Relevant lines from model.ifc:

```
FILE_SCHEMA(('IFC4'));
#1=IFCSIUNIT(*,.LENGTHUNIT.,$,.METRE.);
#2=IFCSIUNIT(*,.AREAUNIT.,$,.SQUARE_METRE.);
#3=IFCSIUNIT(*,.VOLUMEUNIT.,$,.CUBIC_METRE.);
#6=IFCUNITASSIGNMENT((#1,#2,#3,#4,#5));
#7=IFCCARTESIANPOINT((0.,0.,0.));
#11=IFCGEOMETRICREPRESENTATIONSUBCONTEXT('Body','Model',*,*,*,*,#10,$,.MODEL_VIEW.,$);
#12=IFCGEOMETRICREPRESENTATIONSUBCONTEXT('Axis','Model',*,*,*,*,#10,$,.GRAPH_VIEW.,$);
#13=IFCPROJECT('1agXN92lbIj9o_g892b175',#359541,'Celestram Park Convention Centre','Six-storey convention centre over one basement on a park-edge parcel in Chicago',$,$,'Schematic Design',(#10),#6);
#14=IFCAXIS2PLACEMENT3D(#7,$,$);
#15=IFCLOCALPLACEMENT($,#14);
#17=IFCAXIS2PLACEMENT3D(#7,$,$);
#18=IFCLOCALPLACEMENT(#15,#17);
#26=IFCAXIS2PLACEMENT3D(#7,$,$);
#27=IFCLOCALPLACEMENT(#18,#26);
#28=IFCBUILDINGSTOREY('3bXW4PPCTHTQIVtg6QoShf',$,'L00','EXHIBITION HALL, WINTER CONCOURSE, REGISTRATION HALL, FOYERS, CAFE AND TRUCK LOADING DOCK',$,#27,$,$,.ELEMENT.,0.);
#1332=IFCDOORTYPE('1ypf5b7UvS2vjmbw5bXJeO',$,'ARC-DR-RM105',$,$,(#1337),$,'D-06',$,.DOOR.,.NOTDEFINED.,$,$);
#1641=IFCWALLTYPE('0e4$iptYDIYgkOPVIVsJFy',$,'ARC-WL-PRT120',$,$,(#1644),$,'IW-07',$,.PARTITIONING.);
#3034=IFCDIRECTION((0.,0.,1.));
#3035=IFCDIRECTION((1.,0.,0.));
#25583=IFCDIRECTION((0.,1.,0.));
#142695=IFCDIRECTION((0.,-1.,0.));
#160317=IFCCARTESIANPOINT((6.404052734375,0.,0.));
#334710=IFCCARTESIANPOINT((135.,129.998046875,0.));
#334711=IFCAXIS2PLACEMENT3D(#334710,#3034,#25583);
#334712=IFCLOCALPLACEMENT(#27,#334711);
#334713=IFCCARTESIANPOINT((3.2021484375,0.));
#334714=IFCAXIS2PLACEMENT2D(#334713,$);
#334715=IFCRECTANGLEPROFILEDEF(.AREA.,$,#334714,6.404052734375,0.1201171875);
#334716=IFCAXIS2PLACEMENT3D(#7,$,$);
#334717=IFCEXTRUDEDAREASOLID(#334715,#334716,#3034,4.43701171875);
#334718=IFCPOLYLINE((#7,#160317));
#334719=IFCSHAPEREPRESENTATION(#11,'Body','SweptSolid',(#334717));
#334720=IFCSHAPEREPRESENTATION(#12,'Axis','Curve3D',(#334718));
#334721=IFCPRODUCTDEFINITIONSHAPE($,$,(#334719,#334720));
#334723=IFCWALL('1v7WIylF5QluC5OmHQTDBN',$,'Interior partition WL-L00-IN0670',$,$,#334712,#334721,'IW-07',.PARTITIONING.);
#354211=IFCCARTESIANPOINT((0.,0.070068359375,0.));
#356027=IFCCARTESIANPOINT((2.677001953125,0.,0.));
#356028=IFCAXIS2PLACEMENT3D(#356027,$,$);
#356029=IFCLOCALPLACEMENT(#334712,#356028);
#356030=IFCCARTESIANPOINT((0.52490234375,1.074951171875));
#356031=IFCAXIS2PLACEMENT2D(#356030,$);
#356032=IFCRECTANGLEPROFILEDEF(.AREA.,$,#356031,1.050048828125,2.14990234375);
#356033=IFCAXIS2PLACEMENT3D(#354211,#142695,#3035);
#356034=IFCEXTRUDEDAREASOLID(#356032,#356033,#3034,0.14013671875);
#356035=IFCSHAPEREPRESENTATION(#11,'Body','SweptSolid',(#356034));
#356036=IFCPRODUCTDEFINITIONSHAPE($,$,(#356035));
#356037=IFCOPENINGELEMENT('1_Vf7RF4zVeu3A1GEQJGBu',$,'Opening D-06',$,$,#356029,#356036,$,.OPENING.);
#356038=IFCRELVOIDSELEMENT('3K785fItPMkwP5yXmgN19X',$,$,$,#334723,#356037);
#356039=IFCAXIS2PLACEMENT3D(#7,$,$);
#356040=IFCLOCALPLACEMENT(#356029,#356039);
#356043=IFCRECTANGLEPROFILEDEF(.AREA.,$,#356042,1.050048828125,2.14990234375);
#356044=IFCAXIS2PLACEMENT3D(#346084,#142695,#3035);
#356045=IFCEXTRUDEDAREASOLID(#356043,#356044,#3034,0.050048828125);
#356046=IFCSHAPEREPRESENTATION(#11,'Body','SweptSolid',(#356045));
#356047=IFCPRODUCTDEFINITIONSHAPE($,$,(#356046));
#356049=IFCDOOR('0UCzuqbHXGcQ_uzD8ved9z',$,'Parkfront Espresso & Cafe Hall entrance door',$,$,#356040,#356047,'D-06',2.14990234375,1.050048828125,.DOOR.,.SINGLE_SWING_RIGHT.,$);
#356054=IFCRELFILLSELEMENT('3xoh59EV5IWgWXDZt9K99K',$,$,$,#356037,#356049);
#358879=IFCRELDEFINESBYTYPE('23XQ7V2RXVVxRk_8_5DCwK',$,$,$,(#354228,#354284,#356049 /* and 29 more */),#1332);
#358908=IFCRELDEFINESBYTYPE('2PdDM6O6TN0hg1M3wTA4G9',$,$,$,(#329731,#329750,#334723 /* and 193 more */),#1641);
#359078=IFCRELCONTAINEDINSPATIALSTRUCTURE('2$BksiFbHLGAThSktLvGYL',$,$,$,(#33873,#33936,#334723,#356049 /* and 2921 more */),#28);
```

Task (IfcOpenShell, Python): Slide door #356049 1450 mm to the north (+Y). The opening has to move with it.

```python
import ifcopenshell
import ifcopenshell.api.geometry
import ifcopenshell.util.placement

model = ifcopenshell.open("model.ifc")

door = model.by_guid("0UCzuqbHXGcQ_uzD8ved9z")
opening = door.FillsVoids[0].RelatingOpeningElement
wall = opening.VoidsElements[0].RelatingBuildingElement

wall_matrix = ifcopenshell.util.placement.get_local_placement(wall.ObjectPlacement)
shift = wall_matrix[:3, 0] * 1.45
before = ifcopenshell.util.placement.get_local_placement(door.ObjectPlacement)[:3, 3].copy()

# The door is placed relative to its opening, so it follows when the opening moves.
matrix = ifcopenshell.util.placement.get_local_placement(opening.ObjectPlacement)
matrix[:3, 3] += shift
ifcopenshell.api.geometry.edit_object_placement(
    model, product=opening, matrix=matrix, is_si=False, should_transform_children=True
)

after = ifcopenshell.util.placement.get_local_placement(door.ObjectPlacement)[:3, 3]
print("door moved by", (after - before).round(3) + 0.0)

model.write("model_updated.ifc")
```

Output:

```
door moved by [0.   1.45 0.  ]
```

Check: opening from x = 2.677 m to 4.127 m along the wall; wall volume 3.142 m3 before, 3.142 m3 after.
